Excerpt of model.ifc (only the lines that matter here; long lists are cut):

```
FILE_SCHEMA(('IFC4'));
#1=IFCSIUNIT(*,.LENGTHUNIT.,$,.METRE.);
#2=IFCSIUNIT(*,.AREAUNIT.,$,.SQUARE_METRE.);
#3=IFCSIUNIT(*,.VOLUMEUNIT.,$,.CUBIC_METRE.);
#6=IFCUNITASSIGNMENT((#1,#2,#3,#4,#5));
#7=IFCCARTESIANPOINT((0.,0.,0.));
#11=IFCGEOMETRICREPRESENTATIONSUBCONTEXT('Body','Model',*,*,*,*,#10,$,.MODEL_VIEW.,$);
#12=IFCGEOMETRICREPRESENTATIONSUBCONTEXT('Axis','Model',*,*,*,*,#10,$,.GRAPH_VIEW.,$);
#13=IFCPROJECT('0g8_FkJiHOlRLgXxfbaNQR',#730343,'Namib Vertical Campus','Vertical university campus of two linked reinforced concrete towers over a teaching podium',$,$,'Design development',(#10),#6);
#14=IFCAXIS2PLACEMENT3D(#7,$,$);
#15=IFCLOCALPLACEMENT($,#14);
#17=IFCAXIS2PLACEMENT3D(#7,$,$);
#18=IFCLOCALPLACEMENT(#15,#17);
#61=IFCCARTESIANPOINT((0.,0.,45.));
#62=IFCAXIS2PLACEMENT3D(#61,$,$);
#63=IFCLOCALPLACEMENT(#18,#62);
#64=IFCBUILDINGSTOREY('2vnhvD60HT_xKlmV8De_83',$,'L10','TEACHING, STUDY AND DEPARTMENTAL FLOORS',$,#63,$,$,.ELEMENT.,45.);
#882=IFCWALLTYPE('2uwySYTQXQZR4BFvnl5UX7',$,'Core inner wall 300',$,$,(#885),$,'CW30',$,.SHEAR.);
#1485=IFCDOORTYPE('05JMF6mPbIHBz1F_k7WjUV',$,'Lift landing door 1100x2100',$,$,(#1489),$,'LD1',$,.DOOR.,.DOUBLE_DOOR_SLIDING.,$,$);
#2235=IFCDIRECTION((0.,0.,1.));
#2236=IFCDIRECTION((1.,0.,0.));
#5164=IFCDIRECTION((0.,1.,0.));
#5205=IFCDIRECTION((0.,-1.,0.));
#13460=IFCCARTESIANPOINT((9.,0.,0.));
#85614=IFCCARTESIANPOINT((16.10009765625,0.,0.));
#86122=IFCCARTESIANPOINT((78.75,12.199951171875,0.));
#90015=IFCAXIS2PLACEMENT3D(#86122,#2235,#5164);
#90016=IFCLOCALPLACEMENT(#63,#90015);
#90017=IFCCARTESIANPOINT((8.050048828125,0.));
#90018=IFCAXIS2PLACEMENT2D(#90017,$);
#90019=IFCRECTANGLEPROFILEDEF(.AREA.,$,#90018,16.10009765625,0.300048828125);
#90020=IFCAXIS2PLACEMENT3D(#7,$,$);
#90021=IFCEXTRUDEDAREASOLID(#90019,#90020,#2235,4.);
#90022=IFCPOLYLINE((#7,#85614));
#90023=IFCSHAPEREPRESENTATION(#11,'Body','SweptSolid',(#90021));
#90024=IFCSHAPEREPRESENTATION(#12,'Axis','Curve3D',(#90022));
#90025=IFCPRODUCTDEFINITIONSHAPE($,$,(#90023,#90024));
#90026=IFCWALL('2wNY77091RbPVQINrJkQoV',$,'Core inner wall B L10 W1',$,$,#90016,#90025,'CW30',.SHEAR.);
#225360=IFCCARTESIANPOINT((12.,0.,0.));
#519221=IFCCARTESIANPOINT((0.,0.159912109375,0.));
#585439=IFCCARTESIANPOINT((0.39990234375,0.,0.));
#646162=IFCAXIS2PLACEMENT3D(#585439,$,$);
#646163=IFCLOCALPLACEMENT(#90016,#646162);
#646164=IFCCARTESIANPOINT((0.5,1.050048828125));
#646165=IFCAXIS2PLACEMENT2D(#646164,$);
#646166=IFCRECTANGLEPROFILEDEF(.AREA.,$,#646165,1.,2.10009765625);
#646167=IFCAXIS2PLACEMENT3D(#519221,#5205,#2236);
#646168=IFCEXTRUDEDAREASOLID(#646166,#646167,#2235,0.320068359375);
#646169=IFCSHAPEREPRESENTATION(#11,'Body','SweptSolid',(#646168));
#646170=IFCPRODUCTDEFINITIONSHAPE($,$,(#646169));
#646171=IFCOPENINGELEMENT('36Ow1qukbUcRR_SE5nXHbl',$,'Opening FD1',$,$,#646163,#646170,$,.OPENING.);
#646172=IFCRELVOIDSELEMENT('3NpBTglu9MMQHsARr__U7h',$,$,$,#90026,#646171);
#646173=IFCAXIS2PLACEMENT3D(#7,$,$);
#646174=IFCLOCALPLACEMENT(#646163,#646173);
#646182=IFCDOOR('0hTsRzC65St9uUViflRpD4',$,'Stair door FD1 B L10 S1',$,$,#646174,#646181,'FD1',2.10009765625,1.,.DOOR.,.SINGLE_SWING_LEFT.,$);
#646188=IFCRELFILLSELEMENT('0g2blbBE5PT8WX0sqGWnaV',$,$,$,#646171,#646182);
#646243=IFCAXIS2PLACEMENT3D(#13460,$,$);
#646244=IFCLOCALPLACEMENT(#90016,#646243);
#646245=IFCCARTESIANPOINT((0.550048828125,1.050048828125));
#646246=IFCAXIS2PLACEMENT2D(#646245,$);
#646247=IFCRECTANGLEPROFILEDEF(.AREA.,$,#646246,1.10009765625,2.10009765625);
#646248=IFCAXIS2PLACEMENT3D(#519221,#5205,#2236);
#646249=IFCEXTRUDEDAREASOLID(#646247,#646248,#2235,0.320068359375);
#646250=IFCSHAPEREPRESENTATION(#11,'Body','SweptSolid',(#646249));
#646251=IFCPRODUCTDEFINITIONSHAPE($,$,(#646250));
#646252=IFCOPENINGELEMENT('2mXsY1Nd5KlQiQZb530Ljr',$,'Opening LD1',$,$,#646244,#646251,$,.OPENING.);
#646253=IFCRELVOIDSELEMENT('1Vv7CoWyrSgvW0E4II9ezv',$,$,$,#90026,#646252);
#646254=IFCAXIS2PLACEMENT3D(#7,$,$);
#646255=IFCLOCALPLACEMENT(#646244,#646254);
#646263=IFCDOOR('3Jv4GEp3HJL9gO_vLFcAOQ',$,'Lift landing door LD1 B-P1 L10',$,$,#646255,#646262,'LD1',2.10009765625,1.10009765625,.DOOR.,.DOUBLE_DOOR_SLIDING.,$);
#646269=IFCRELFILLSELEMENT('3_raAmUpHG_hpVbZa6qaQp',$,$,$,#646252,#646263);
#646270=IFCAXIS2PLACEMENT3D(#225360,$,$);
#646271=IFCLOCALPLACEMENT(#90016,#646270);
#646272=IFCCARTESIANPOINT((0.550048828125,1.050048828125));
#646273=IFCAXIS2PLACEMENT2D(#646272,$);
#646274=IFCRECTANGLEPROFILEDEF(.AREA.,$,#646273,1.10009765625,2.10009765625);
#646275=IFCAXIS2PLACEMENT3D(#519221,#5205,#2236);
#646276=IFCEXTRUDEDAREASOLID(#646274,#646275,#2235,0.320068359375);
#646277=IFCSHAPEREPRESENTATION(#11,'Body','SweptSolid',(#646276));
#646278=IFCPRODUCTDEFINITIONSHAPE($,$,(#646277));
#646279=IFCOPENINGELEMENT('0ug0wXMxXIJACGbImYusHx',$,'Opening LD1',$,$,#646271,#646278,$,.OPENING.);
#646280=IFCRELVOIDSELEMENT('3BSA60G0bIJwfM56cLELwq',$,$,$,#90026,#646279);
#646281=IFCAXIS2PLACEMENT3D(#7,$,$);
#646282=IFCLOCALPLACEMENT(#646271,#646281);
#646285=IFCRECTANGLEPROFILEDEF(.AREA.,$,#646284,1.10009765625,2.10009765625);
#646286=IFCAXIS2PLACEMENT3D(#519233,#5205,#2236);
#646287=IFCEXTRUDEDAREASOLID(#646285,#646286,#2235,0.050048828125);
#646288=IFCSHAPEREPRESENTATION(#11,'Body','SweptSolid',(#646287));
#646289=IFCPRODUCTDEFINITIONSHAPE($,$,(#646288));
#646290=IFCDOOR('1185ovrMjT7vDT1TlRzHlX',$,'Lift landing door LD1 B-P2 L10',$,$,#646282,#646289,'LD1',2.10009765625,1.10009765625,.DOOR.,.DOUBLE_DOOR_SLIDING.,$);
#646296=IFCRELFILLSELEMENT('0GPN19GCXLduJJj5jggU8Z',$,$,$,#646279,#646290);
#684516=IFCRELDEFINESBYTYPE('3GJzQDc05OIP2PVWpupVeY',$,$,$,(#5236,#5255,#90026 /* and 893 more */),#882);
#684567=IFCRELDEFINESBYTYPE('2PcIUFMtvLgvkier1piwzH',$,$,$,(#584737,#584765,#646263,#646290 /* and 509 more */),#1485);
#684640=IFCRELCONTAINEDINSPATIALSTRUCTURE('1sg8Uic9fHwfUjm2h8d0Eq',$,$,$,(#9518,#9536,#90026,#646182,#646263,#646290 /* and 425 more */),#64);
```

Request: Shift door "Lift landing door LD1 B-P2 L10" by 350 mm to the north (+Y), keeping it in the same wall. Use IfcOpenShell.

```python
import ifcopenshell
import ifcopenshell.api.geometry
import ifcopenshell.util.placement
import ifcopenshell.util.unit

model = ifcopenshell.open("model.ifc")
unit_scale = ifcopenshell.util.unit.calculate_unit_scale(model)

door = model.by_guid("1185ovrMjT7vDT1TlRzHlX")
opening = door.FillsVoids[0].RelatingOpeningElement
wall = opening.VoidsElements[0].RelatingBuildingElement

wall_matrix = ifcopenshell.util.placement.get_local_placement(wall.ObjectPlacement)
shift = wall_matrix[:3, 0] * 0.35 / unit_scale
before = ifcopenshell.util.placement.get_local_placement(door.ObjectPlacement)[:3, 3].copy()

# The door is placed relative to its opening, so it follows when the opening moves.
matrix = ifcopenshell.util.placement.get_local_placement(opening.ObjectPlacement)
matrix[:3, 3] += shift
ifcopenshell.api.geometry.edit_object_placement(
    model, product=opening, matrix=matrix, is_si=False, should_transform_children=True
)

after = ifcopenshell.util.placement.get_local_placement(door.ObjectPlacement)[:3, 3]
print("door moved by", (after - before).round(3) + 0.0)

model.write("model-out.ifc")
```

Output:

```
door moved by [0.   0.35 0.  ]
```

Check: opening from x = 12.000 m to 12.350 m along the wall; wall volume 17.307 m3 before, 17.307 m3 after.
